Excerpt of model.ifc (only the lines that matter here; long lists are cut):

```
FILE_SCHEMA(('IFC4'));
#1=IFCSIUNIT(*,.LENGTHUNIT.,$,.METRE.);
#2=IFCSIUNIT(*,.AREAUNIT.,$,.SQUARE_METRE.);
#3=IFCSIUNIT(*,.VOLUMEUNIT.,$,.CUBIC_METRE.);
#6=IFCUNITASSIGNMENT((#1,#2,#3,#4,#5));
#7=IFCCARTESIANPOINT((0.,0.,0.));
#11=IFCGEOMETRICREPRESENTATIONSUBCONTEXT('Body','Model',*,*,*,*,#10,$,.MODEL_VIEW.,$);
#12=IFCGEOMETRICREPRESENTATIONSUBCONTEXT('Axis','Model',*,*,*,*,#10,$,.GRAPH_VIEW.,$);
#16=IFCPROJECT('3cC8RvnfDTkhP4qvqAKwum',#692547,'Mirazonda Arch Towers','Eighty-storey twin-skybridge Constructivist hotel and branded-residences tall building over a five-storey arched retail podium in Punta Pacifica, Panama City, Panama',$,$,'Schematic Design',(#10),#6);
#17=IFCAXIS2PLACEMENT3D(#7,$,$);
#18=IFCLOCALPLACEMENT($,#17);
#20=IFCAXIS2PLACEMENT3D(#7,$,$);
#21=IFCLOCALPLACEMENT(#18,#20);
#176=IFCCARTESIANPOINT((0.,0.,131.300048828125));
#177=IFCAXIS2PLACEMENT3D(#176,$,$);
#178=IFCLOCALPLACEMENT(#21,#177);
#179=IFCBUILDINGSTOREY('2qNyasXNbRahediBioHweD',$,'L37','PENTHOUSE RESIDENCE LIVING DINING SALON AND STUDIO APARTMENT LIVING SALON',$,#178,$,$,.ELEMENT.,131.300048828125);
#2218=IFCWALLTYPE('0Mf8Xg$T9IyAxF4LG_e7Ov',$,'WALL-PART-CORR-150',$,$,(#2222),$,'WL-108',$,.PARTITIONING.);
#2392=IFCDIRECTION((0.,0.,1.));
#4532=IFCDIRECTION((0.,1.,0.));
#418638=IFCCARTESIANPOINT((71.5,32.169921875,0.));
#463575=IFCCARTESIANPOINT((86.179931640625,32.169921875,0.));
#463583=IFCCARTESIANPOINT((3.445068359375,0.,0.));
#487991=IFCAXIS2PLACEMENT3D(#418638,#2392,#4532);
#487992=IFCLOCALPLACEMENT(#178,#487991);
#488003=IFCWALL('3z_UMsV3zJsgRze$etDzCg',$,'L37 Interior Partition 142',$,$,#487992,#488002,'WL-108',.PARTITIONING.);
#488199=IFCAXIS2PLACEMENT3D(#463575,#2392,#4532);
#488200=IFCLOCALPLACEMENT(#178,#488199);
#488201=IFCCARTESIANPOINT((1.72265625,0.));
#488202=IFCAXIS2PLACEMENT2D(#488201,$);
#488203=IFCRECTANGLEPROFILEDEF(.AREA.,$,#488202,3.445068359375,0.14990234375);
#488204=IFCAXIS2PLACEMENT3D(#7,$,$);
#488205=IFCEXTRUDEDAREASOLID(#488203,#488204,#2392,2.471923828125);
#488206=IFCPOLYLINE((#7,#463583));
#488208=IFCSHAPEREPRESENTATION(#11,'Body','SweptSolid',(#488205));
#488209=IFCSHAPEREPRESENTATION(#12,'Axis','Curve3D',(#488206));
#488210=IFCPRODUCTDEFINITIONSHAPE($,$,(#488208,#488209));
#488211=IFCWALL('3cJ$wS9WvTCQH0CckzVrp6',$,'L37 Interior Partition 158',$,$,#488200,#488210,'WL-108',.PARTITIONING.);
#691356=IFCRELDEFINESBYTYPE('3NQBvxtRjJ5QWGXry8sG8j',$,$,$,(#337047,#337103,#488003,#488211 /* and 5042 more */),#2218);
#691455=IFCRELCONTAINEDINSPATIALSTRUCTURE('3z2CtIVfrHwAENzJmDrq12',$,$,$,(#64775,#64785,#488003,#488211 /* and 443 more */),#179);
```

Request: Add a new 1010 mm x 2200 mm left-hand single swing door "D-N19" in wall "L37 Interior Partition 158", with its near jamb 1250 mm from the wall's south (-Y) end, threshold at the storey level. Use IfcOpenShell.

```python
import numpy as np
import ifcopenshell
import ifcopenshell.api.feature
import ifcopenshell.api.geometry
import ifcopenshell.api.root
import ifcopenshell.api.spatial
import ifcopenshell.geom
import ifcopenshell.util.element
import ifcopenshell.util.placement
import ifcopenshell.util.representation
import ifcopenshell.util.shape
import ifcopenshell.util.unit

model = ifcopenshell.open("model.ifc")
unit_scale = ifcopenshell.util.unit.calculate_unit_scale(model)
settings = ifcopenshell.geom.settings()


def volume(element):
    """Net volume in cubic metres, openings subtracted."""
    shape = ifcopenshell.geom.create_shape(settings, element)
    return ifcopenshell.util.shape.get_volume(shape.geometry)


wall = model.by_guid("3cJ$wS9WvTCQH0CckzVrp6")
storey = ifcopenshell.util.element.get_container(wall, ifc_class="IfcBuildingStorey")
context = ifcopenshell.util.representation.get_context(model, "Model", "Body", "MODEL_VIEW")
before = volume(wall)

width, height, from_end, sill = 1.01, 2.2, 1.25, 0.0  # metres

# The wall runs along its own X axis, and the end named is its -X end.
wall_shape = ifcopenshell.geom.create_shape(settings, wall)
x, y, z = ifcopenshell.util.shape.get_vertices(wall_shape.geometry).T
start = x.min() + from_end
face, thickness = float(y.min()), float(y.max() - y.min())
wall_matrix = ifcopenshell.util.placement.get_local_placement(wall.ObjectPlacement)
level = ifcopenshell.util.placement.get_local_placement(storey.ObjectPlacement)[2, 3]


def in_wall(x, y):
    """Placement at x, y metres in the wall's axes, at sill height."""
    matrix = wall_matrix.copy()
    matrix[:, 3] = wall_matrix @ np.array([x / unit_scale, y / unit_scale, 0.0, 1.0])
    matrix[2, 3] = level + sill / unit_scale
    return matrix


# Opening: a box that overshoots both wall faces by 50 mm.
opening = ifcopenshell.api.root.create_entity(model, ifc_class="IfcOpeningElement", predefined_type="OPENING")
box = ifcopenshell.api.geometry.add_wall_representation(
    model, context=context, length=width, height=height, thickness=thickness + 0.1
)
ifcopenshell.api.geometry.assign_representation(model, product=opening, representation=box)
ifcopenshell.api.geometry.edit_object_placement(model, product=opening, matrix=in_wall(start, face - 0.05), is_si=False)
ifcopenshell.api.feature.add_feature(model, feature=opening, element=wall)

door = ifcopenshell.api.root.create_entity(model, ifc_class="IfcDoor", name="D-N19", predefined_type="DOOR")
door.OverallWidth, door.OverallHeight = width / unit_scale, height / unit_scale
door.OperationType = "SINGLE_SWING_LEFT"
body = ifcopenshell.api.geometry.add_door_representation(
    model,
    context=context,
    overall_width=door.OverallWidth,
    overall_height=door.OverallHeight,
    operation_type="SINGLE_SWING_LEFT",
    lining_properties={"LiningDepth": thickness / unit_scale, "ThresholdDepth": thickness / unit_scale},
)
ifcopenshell.api.geometry.assign_representation(model, product=door, representation=body)
ifcopenshell.api.spatial.assign_container(model, products=[door], relating_structure=storey)
ifcopenshell.api.feature.add_filling(model, opening=opening, element=door)

# The lining spans the wall, so the door starts at the wall face.
ifcopenshell.api.geometry.edit_object_placement(model, product=door, matrix=in_wall(start, face), is_si=False)

after = volume(wall)

print(f"wall volume {before:.3f} -> {after:.3f} m3")

model.write("model_updated.ifc")
```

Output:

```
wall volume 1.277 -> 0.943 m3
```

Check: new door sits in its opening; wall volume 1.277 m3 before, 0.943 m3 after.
